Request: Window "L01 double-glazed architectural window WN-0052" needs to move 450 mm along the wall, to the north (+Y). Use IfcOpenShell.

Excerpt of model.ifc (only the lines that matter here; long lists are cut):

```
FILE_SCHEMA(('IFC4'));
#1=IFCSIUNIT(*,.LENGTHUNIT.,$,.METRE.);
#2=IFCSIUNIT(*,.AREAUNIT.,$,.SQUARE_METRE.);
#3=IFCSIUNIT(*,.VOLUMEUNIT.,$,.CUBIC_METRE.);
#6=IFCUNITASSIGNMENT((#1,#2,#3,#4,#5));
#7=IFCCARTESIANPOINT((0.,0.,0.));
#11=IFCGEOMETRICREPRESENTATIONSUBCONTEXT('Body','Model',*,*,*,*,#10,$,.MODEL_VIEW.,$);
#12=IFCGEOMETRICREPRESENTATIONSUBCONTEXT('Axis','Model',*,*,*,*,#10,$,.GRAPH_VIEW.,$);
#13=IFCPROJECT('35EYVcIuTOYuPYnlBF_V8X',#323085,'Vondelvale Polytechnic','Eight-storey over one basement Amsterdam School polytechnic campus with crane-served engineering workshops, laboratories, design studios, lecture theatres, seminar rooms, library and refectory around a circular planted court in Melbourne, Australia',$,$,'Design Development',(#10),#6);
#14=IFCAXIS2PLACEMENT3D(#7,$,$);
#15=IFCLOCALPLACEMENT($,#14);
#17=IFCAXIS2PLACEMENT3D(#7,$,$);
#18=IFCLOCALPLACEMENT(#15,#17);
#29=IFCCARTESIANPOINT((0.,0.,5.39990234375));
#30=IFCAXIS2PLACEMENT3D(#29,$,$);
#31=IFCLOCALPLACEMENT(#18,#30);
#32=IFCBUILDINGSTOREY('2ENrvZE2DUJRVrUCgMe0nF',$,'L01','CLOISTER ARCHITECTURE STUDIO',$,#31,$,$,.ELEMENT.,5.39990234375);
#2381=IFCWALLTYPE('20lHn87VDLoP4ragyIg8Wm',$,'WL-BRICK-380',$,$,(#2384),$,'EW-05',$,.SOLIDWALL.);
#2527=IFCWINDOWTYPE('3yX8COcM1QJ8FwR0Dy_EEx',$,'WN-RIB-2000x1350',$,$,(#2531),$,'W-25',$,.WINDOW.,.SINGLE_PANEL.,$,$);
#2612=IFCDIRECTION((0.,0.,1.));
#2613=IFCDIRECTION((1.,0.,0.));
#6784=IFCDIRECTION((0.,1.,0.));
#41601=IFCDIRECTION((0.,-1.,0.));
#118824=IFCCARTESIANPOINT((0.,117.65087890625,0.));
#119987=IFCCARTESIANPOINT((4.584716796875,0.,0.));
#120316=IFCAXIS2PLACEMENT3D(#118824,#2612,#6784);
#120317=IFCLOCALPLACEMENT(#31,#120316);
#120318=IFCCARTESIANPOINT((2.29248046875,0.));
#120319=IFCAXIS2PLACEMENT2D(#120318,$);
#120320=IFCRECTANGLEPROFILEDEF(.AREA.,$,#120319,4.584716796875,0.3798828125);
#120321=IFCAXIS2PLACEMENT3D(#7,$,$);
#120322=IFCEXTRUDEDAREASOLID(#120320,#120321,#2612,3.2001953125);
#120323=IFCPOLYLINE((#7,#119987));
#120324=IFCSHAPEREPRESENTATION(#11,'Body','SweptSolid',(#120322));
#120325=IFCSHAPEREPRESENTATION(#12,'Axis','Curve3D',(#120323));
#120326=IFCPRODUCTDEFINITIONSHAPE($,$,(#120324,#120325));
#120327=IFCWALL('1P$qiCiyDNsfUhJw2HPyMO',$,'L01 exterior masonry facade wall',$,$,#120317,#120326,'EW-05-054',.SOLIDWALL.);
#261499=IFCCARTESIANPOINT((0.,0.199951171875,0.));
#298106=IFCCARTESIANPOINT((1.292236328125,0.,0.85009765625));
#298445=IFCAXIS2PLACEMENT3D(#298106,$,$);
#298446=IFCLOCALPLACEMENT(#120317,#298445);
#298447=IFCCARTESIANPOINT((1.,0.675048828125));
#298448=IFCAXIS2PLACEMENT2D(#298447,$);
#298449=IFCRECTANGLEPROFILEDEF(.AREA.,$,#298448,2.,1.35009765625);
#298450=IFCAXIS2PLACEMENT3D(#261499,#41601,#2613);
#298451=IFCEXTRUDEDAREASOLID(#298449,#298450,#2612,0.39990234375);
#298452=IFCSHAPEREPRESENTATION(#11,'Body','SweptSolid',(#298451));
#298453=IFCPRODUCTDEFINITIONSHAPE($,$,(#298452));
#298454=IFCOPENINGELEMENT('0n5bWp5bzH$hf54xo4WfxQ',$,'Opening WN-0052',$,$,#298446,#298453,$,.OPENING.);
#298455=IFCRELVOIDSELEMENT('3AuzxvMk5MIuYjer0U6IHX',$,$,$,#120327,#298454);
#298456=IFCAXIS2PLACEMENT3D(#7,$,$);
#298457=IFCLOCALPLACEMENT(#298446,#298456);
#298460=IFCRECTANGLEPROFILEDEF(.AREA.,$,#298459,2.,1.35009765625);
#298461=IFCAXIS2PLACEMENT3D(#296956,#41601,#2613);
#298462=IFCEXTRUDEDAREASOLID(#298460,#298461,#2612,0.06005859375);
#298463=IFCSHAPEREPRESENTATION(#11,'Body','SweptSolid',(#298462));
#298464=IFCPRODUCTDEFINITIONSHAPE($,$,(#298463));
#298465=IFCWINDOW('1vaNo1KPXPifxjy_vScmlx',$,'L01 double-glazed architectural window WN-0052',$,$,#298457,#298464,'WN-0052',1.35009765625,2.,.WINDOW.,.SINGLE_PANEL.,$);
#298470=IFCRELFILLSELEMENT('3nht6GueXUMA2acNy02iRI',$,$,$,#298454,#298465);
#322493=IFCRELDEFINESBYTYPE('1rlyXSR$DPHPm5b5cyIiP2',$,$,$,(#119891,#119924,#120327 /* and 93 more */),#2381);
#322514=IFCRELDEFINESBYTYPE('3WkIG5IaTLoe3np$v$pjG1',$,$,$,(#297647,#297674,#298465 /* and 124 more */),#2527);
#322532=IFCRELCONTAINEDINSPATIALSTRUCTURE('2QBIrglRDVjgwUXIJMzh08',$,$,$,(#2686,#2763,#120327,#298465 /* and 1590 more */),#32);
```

```python
import ifcopenshell
import ifcopenshell.api.geometry
import ifcopenshell.util.placement

model = ifcopenshell.open("model.ifc")

window = model.by_id(298465)
opening = window.FillsVoids[0].RelatingOpeningElement
wall = opening.VoidsElements[0].RelatingBuildingElement

wall_matrix = ifcopenshell.util.placement.get_local_placement(wall.ObjectPlacement)
shift = wall_matrix[:3, 0] * 0.45
before = ifcopenshell.util.placement.get_local_placement(window.ObjectPlacement)[:3, 3].copy()

# The window is placed relative to its opening, so it follows when the opening moves.
matrix = ifcopenshell.util.placement.get_local_placement(opening.ObjectPlacement)
matrix[:3, 3] += shift
ifcopenshell.api.geometry.edit_object_placement(
    model, product=opening, matrix=matrix, is_si=False, should_transform_children=True
)

after = ifcopenshell.util.placement.get_local_placement(window.ObjectPlacement)[:3, 3]
print("window moved by", (after - before).round(3) + 0.0)

model.write("model_updated.ifc")
```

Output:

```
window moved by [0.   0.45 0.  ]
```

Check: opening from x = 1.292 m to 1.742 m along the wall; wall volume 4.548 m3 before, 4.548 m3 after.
